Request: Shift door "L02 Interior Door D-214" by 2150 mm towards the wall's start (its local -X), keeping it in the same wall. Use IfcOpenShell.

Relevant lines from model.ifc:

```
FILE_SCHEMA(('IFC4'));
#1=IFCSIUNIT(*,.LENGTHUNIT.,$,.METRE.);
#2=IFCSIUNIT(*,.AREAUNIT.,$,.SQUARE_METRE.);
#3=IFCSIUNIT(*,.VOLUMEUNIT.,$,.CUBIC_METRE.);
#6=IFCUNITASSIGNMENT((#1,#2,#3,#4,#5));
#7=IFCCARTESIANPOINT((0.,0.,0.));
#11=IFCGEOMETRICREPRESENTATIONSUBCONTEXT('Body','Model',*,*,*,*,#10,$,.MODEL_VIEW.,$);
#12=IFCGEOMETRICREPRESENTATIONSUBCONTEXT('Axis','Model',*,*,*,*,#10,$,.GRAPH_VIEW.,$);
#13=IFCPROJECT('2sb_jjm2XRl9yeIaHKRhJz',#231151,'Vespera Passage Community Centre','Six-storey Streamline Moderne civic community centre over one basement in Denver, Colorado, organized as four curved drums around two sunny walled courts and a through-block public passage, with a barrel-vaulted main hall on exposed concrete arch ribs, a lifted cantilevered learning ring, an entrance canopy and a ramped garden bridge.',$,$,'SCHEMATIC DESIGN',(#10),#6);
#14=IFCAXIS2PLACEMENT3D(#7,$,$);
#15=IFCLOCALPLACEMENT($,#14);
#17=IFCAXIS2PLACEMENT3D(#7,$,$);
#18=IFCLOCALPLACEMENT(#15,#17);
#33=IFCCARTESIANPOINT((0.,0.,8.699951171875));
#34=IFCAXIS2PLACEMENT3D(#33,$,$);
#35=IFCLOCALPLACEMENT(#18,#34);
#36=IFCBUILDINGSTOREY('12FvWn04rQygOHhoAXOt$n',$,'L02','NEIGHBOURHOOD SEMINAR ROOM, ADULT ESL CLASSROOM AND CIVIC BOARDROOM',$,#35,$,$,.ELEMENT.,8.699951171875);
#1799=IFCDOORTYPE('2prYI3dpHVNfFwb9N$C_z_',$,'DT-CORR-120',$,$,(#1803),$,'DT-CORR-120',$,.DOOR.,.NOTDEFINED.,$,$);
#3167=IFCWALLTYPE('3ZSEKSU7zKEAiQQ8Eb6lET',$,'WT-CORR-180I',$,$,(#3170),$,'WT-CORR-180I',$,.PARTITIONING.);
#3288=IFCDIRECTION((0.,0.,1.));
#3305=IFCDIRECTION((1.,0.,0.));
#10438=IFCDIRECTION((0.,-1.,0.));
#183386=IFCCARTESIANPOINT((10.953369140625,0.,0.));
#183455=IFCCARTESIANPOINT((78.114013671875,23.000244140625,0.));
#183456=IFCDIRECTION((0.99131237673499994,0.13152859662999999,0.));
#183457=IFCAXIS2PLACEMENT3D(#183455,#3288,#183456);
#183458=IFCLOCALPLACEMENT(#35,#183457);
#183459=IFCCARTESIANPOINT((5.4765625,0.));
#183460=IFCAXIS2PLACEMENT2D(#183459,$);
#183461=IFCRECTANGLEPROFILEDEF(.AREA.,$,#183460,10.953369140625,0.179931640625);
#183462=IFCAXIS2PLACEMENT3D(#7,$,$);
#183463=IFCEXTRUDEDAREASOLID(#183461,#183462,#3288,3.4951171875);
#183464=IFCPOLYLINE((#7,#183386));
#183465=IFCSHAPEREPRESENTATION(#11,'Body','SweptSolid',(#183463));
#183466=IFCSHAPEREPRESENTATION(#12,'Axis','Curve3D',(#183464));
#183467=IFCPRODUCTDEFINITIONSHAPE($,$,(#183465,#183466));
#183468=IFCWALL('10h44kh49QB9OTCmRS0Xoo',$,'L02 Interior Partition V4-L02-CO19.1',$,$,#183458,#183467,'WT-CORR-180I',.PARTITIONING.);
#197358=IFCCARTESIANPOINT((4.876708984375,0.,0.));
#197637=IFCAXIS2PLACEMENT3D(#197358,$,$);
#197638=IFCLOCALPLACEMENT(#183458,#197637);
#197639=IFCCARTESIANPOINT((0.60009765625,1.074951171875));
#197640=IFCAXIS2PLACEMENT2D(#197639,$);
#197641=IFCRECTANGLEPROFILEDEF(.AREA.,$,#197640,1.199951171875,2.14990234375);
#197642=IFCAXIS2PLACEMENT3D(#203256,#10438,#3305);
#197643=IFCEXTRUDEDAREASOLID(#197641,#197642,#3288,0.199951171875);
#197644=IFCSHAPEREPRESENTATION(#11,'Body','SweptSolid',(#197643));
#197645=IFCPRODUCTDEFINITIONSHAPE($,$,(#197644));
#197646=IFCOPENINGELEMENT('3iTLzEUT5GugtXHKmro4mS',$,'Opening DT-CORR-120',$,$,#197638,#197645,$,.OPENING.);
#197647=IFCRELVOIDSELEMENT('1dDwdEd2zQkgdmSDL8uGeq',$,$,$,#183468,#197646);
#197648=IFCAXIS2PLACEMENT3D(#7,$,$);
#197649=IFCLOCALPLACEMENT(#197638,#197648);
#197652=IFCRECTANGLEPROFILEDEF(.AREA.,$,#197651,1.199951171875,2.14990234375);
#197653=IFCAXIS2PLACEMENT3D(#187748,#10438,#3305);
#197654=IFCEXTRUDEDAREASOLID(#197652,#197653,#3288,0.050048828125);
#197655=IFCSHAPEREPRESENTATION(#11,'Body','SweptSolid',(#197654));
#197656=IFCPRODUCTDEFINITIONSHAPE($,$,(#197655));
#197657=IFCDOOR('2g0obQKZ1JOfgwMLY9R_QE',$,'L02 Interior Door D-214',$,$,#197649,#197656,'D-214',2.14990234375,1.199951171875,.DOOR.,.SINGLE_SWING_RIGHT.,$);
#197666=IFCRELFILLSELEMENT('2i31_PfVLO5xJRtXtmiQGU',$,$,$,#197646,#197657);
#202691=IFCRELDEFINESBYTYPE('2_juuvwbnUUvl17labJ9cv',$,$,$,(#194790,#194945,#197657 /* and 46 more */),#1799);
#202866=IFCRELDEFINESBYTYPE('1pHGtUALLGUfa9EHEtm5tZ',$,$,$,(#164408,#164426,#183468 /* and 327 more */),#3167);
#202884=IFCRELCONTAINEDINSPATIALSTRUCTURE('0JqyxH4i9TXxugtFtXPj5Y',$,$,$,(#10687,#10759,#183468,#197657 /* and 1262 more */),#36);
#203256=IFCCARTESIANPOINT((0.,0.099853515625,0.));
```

```python
import ifcopenshell
import ifcopenshell.api.geometry
import ifcopenshell.util.placement
import ifcopenshell.util.unit

model = ifcopenshell.open("model.ifc")
unit_scale = ifcopenshell.util.unit.calculate_unit_scale(model)

door = model.by_guid("2g0obQKZ1JOfgwMLY9R_QE")
opening = door.FillsVoids[0].RelatingOpeningElement
wall = opening.VoidsElements[0].RelatingBuildingElement

wall_matrix = ifcopenshell.util.placement.get_local_placement(wall.ObjectPlacement)
shift = wall_matrix[:3, 0] * -2.15 / unit_scale
before = ifcopenshell.util.placement.get_local_placement(door.ObjectPlacement)[:3, 3].copy()

# The door is placed relative to its opening, so it follows when the opening moves.
matrix = ifcopenshell.util.placement.get_local_placement(opening.ObjectPlacement)
matrix[:3, 3] += shift
ifcopenshell.api.geometry.edit_object_placement(
    model, product=opening, matrix=matrix, is_si=False, should_transform_children=True
)

after = ifcopenshell.util.placement.get_local_placement(door.ObjectPlacement)[:3, 3]
print("door moved by", (after - before).round(3) + 0.0)

model.write("model_updated.ifc")
```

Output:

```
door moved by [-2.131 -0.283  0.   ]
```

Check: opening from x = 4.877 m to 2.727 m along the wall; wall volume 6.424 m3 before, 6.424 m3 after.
